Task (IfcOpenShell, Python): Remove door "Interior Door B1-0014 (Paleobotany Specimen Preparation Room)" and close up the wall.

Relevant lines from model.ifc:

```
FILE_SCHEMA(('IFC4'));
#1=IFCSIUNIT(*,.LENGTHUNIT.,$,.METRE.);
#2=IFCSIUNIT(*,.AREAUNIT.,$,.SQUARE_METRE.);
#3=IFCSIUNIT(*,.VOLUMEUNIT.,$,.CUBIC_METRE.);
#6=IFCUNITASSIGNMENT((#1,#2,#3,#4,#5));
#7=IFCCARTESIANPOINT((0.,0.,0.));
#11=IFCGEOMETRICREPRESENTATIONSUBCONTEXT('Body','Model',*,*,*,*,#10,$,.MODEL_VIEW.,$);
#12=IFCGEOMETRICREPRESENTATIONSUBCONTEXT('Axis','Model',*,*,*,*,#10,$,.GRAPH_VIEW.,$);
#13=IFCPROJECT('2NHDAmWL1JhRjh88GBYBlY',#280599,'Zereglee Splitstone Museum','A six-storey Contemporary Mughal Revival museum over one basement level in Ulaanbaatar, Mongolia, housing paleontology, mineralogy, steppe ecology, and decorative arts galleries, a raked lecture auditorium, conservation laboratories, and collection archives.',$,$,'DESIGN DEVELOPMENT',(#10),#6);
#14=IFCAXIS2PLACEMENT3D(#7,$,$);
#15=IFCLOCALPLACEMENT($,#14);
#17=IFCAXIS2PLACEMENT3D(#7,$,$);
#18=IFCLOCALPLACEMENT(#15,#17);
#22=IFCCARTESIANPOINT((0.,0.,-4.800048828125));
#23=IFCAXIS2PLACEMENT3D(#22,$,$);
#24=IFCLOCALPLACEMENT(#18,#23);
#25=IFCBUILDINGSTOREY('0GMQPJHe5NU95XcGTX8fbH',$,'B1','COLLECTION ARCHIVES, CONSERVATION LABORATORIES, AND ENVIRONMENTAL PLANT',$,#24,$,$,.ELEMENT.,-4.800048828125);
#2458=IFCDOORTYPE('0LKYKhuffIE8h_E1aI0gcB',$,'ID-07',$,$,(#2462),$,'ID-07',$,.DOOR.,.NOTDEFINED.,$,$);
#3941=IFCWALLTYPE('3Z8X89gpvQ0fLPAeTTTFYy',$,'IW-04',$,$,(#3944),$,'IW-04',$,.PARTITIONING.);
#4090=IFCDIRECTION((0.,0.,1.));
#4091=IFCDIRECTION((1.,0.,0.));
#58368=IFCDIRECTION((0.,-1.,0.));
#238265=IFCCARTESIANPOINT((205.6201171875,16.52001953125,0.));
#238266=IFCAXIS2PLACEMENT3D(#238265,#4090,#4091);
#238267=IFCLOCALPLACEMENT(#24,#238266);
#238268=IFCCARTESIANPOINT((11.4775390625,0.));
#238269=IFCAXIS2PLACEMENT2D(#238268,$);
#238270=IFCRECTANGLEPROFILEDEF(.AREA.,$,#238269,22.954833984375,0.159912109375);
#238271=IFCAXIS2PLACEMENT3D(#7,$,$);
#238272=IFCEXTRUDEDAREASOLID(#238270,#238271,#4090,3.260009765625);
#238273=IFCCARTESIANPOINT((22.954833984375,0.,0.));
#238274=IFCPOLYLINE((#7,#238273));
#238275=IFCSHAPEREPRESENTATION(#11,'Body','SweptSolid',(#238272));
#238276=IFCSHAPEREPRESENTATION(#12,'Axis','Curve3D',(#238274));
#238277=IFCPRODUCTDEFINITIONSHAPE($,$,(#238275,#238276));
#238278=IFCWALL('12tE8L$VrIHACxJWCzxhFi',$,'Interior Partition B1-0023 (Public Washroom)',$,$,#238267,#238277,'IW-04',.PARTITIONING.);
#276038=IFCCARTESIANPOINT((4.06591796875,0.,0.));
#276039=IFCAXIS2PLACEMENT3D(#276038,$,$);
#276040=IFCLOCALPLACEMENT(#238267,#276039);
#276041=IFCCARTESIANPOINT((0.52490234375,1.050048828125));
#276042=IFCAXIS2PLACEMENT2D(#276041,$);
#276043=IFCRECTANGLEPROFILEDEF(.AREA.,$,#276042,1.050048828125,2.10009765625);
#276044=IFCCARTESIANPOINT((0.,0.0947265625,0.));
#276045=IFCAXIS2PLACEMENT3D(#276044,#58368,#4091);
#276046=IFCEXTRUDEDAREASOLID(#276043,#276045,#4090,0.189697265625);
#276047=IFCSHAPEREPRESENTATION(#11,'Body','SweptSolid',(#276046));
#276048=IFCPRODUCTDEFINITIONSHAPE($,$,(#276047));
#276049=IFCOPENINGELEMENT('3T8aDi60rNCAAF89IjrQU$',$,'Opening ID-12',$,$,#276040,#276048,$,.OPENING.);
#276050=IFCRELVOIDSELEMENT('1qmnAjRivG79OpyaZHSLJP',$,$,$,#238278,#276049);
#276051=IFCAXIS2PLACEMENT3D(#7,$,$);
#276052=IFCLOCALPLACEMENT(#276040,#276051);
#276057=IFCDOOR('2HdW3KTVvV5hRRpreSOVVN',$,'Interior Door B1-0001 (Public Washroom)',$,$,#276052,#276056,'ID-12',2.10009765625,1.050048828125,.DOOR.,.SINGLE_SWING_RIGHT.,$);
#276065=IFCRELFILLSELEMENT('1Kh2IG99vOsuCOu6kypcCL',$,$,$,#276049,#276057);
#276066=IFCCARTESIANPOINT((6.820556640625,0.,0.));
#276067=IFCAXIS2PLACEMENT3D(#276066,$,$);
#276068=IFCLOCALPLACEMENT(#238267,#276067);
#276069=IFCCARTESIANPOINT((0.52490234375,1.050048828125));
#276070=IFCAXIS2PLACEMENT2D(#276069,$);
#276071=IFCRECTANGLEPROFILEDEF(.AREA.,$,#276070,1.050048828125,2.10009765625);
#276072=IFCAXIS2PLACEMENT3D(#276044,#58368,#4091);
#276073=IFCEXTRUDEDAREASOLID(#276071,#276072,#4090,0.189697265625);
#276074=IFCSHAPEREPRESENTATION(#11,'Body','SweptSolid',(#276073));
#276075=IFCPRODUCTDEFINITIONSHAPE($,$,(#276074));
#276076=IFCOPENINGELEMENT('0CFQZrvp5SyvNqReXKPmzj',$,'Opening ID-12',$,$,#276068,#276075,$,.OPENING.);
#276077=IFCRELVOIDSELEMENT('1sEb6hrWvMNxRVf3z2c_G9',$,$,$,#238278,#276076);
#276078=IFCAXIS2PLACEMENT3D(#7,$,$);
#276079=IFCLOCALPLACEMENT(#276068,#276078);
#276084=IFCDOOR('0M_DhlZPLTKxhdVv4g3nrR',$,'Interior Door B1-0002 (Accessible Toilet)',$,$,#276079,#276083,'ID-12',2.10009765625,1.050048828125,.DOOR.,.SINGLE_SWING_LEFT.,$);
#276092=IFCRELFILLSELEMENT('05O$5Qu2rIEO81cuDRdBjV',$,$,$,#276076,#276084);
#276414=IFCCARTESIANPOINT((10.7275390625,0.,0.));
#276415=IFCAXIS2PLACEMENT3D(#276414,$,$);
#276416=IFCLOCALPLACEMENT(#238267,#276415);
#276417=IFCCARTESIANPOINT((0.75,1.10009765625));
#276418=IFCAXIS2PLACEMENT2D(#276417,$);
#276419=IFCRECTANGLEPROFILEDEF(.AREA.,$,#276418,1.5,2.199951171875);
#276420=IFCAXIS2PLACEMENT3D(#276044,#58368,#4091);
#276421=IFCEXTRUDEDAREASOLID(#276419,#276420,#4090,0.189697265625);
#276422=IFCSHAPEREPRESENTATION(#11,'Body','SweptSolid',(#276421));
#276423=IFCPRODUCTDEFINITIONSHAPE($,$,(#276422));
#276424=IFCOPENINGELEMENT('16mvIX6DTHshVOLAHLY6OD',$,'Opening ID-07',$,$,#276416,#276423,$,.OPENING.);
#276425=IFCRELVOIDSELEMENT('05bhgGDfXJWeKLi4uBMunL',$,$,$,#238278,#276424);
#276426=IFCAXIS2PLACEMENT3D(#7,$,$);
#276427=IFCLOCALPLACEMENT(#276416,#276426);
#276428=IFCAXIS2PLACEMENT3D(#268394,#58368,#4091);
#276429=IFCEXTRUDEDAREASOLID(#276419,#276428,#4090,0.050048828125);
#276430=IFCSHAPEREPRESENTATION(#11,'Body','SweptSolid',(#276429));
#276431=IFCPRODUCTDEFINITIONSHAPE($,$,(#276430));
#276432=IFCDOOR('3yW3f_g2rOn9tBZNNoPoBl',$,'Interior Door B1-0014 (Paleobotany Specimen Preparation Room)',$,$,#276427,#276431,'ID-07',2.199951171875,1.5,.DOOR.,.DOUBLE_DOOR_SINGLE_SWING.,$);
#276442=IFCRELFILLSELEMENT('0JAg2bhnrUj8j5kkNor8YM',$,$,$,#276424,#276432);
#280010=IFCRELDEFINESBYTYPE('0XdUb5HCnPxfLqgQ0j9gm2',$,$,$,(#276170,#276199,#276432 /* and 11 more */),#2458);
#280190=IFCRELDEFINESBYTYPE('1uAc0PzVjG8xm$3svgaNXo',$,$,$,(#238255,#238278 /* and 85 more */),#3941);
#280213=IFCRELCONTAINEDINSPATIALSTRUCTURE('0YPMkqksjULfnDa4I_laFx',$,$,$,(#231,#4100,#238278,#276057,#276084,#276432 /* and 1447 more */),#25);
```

```python
import ifcopenshell
import ifcopenshell.api.feature
import ifcopenshell.api.root
import ifcopenshell.geom
import ifcopenshell.util.shape

model = ifcopenshell.open("model.ifc")
settings = ifcopenshell.geom.settings()


def volume(element):
    """Net volume in cubic metres, openings subtracted."""
    shape = ifcopenshell.geom.create_shape(settings, element)
    return ifcopenshell.util.shape.get_volume(shape.geometry)


door = model.by_guid("3yW3f_g2rOn9tBZNNoPoBl")
opening = door.FillsVoids[0].RelatingOpeningElement
wall = opening.VoidsElements[0].RelatingBuildingElement
before = volume(wall)

ifcopenshell.api.root.remove_product(model, product=door)
ifcopenshell.api.feature.remove_feature(model, feature=opening)

after = volume(wall)

print(f"wall volume {before:.3f} -> {after:.3f} m3")

model.write("model_v2.ifc")
```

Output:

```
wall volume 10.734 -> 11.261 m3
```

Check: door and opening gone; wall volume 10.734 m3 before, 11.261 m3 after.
